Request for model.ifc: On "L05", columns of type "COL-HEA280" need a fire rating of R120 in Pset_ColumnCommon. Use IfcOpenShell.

First a look at what the model holds.

```python
import ifcopenshell
import ifcopenshell.util.element

model = ifcopenshell.open("model.ifc")
print(model.schema)
storey = next(s for s in model.by_type("IfcBuildingStorey") if s.Name == "L05")
columns = [e for e in ifcopenshell.util.element.get_decomposition(storey) if e.is_a("IfcColumn")]
seen = {}
for e in columns:
    element_type = ifcopenshell.util.element.get_type(e)
    key = (element_type.Name if element_type != e and element_type else None, ifcopenshell.util.element.get_pset(e, "Pset_ColumnCommon", "FireRating"))
    seen[key] = seen.get(key, 0) + 1
for (name, value), count in sorted(seen.items(), key=str):
    print(count, "x", name, "|", value)
```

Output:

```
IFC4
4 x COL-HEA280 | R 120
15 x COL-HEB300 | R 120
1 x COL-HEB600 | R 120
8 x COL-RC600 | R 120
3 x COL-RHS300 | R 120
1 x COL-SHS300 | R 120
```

```python
import ifcopenshell
import ifcopenshell.api.pset
import ifcopenshell.util.element

model = ifcopenshell.open("model.ifc")

storey = next(s for s in model.by_type("IfcBuildingStorey") if s.Name == "L05")
columns = [e for e in ifcopenshell.util.element.get_decomposition(storey) if e.is_a("IfcColumn")]

count = 0
for e in columns:
    element_type = ifcopenshell.util.element.get_type(e)
    if element_type in (None, e) or element_type.Name != "COL-HEA280":
        continue
    # add_pset returns the element's existing set when there is one.
    pset = ifcopenshell.api.pset.add_pset(model, product=e, name="Pset_ColumnCommon")
    ifcopenshell.api.pset.edit_pset(model, pset=pset, properties={"FireRating": "R120"})
    count += 1

print(count, "columns updated")

model.write("model_edited.ifc")
```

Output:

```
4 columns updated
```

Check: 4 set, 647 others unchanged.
